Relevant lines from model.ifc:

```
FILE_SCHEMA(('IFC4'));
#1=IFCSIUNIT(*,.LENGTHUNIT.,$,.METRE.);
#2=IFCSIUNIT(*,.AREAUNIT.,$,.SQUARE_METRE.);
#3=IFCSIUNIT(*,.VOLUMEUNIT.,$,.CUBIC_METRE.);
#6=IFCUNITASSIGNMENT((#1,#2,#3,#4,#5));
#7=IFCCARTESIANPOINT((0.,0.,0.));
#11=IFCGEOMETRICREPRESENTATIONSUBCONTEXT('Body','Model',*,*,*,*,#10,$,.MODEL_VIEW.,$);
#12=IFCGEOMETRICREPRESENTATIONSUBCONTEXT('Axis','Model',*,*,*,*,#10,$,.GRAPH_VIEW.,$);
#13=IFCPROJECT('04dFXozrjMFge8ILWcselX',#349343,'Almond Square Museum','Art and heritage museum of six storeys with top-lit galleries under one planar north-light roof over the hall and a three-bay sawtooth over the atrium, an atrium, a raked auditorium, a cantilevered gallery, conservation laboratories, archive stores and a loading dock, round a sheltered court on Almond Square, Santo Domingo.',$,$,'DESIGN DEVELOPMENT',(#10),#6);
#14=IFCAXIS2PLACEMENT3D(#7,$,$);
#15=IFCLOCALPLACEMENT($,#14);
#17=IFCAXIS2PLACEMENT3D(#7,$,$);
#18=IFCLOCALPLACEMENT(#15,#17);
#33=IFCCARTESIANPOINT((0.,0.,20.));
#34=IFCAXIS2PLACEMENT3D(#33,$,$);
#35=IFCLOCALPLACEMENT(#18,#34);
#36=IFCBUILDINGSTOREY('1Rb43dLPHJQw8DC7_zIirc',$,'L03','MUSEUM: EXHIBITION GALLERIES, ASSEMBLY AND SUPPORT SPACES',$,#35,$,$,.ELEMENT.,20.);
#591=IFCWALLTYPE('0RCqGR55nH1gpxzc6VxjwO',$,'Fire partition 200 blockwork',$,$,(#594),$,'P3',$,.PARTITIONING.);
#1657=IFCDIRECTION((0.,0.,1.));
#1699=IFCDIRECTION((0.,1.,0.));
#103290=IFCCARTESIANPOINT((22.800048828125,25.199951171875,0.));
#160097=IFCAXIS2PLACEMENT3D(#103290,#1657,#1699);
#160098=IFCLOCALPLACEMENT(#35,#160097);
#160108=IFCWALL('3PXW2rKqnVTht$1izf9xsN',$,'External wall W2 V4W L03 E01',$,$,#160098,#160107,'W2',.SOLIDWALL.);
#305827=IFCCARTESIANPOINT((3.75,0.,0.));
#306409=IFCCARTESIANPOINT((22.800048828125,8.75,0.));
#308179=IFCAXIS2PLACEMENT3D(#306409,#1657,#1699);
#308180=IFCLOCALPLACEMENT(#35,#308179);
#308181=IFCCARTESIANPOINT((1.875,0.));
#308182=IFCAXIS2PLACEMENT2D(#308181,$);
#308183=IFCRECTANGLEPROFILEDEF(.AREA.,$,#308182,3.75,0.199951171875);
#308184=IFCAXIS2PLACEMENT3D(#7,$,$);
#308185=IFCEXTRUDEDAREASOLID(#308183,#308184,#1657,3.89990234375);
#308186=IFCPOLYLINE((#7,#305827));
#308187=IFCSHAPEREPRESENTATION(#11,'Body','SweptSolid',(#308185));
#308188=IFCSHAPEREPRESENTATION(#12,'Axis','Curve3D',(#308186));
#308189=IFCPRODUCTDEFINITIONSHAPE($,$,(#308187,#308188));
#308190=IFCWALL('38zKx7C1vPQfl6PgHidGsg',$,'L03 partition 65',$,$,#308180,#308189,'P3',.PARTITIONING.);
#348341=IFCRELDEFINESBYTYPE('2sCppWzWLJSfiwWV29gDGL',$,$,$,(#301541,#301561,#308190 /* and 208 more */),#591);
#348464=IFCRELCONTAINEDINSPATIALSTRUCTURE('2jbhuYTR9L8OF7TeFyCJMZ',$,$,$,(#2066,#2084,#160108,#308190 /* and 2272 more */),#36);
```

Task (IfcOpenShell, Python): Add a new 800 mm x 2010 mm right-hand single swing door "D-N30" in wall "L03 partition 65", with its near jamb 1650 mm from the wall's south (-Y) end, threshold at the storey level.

```python
import numpy as np
import ifcopenshell
import ifcopenshell.api.feature
import ifcopenshell.api.geometry
import ifcopenshell.api.root
import ifcopenshell.api.spatial
import ifcopenshell.geom
import ifcopenshell.util.element
import ifcopenshell.util.placement
import ifcopenshell.util.representation
import ifcopenshell.util.shape
import ifcopenshell.util.unit

model = ifcopenshell.open("model.ifc")
unit_scale = ifcopenshell.util.unit.calculate_unit_scale(model)
settings = ifcopenshell.geom.settings()


def volume(element):
    """Net volume in cubic metres, openings subtracted."""
    shape = ifcopenshell.geom.create_shape(settings, element)
    return ifcopenshell.util.shape.get_volume(shape.geometry)


wall = model.by_id(308190)
storey = ifcopenshell.util.element.get_container(wall, ifc_class="IfcBuildingStorey")
context = ifcopenshell.util.representation.get_context(model, "Model", "Body", "MODEL_VIEW")
before = volume(wall)

width, height, from_end, sill = 0.8, 2.01, 1.65, 0.0  # metres

# The wall runs along its own X axis, and the end named is its -X end.
wall_shape = ifcopenshell.geom.create_shape(settings, wall)
x, y, z = ifcopenshell.util.shape.get_vertices(wall_shape.geometry).T
start = x.min() + from_end
face, thickness = float(y.min()), float(y.max() - y.min())
wall_matrix = ifcopenshell.util.placement.get_local_placement(wall.ObjectPlacement)
level = ifcopenshell.util.placement.get_local_placement(storey.ObjectPlacement)[2, 3]


def in_wall(x, y):
    """Placement at x, y metres in the wall's axes, at sill height."""
    matrix = wall_matrix.copy()
    matrix[:, 3] = wall_matrix @ np.array([x / unit_scale, y / unit_scale, 0.0, 1.0])
    matrix[2, 3] = level + sill / unit_scale
    return matrix


# Opening: a box that overshoots both wall faces by 50 mm.
opening = ifcopenshell.api.root.create_entity(model, ifc_class="IfcOpeningElement", predefined_type="OPENING")
box = ifcopenshell.api.geometry.add_wall_representation(
    model, context=context, length=width, height=height, thickness=thickness + 0.1
)
ifcopenshell.api.geometry.assign_representation(model, product=opening, representation=box)
ifcopenshell.api.geometry.edit_object_placement(model, product=opening, matrix=in_wall(start, face - 0.05), is_si=False)
ifcopenshell.api.feature.add_feature(model, feature=opening, element=wall)

door = ifcopenshell.api.root.create_entity(model, ifc_class="IfcDoor", name="D-N30", predefined_type="DOOR")
door.OverallWidth, door.OverallHeight = width / unit_scale, height / unit_scale
door.OperationType = "SINGLE_SWING_RIGHT"
body = ifcopenshell.api.geometry.add_door_representation(
    model,
    context=context,
    overall_width=door.OverallWidth,
    overall_height=door.OverallHeight,
    operation_type="SINGLE_SWING_RIGHT",
    lining_properties={"LiningDepth": thickness / unit_scale, "ThresholdDepth": thickness / unit_scale},
)
ifcopenshell.api.geometry.assign_representation(model, product=door, representation=body)
ifcopenshell.api.spatial.assign_container(model, products=[door], relating_structure=storey)
ifcopenshell.api.feature.add_filling(model, opening=opening, element=door)

# The lining spans the wall, so the door starts at the wall face.
ifcopenshell.api.geometry.edit_object_placement(model, product=door, matrix=in_wall(start, face), is_si=False)

after = volume(wall)

print(f"wall volume {before:.3f} -> {after:.3f} m3")

model.write("model_v2.ifc")
```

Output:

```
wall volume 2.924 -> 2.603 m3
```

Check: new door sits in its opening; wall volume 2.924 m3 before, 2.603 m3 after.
